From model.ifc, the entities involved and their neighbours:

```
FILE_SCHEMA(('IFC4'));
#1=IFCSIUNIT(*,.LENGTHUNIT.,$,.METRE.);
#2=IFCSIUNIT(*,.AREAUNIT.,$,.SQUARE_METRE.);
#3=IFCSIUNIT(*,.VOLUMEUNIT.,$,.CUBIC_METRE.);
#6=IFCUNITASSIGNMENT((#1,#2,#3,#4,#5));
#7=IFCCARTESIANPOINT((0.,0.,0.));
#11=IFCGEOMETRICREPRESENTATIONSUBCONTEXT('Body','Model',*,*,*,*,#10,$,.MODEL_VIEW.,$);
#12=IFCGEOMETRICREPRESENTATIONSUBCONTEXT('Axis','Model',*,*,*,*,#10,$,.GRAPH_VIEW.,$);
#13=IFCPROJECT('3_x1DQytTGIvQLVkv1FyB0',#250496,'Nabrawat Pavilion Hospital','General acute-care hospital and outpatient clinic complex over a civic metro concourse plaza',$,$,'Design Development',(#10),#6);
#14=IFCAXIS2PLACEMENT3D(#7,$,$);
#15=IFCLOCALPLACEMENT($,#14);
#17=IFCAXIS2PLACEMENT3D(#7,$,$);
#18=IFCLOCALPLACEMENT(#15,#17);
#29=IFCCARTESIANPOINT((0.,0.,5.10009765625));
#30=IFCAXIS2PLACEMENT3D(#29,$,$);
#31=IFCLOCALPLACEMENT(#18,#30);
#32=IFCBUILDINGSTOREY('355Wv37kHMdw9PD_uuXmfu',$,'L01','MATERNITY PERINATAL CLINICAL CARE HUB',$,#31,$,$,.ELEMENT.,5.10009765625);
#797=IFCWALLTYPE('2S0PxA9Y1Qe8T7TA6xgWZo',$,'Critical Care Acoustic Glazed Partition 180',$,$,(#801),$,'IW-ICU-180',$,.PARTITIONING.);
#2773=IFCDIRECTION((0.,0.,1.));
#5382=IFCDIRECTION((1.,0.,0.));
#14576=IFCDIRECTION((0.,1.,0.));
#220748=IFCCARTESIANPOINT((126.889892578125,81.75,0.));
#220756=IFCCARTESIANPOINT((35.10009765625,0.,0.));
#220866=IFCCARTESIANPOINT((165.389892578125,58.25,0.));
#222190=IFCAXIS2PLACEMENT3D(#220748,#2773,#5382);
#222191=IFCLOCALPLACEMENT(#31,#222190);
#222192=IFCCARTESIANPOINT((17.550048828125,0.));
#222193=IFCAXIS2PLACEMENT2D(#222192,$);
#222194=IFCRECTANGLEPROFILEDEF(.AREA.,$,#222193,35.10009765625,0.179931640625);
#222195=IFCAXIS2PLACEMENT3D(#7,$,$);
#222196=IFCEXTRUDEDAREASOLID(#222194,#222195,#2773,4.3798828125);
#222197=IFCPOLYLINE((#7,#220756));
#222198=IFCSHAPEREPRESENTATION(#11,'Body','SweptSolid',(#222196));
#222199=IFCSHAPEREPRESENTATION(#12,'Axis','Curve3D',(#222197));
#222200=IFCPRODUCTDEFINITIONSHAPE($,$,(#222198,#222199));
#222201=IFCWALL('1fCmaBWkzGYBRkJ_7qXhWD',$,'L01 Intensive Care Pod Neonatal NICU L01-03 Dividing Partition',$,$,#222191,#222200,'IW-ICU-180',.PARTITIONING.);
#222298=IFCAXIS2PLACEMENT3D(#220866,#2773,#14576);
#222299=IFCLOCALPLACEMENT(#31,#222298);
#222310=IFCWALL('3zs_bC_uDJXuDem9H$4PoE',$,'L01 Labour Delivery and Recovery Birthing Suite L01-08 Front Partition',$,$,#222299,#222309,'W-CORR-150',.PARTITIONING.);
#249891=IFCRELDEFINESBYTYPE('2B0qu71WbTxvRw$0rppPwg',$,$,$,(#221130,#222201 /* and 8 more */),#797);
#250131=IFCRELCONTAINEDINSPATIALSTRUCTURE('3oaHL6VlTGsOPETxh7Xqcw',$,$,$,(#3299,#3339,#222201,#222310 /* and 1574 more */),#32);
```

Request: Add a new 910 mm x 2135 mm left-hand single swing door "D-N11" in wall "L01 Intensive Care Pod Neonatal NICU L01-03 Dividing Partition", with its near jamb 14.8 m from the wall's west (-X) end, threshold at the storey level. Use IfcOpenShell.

```python
import numpy as np
import ifcopenshell
import ifcopenshell.api.feature
import ifcopenshell.api.geometry
import ifcopenshell.api.root
import ifcopenshell.api.spatial
import ifcopenshell.geom
import ifcopenshell.util.element
import ifcopenshell.util.placement
import ifcopenshell.util.representation
import ifcopenshell.util.shape
import ifcopenshell.util.unit

model = ifcopenshell.open("model.ifc")
unit_scale = ifcopenshell.util.unit.calculate_unit_scale(model)
settings = ifcopenshell.geom.settings()


def volume(element):
    """Net volume in cubic metres, openings subtracted."""
    shape = ifcopenshell.geom.create_shape(settings, element)
    return ifcopenshell.util.shape.get_volume(shape.geometry)


wall = model.by_guid("1fCmaBWkzGYBRkJ_7qXhWD")
storey = ifcopenshell.util.element.get_container(wall, ifc_class="IfcBuildingStorey")
context = ifcopenshell.util.representation.get_context(model, "Model", "Body", "MODEL_VIEW")
before = volume(wall)

width, height, from_end, sill = 0.91, 2.135, 14.8, 0.0  # metres

# The wall runs along its own X axis, and the end named is its -X end.
wall_shape = ifcopenshell.geom.create_shape(settings, wall)
x, y, z = ifcopenshell.util.shape.get_vertices(wall_shape.geometry).T
start = x.min() + from_end
face, thickness = float(y.min()), float(y.max() - y.min())
wall_matrix = ifcopenshell.util.placement.get_local_placement(wall.ObjectPlacement)
level = ifcopenshell.util.placement.get_local_placement(storey.ObjectPlacement)[2, 3]


def in_wall(x, y):
    """Placement at x, y metres in the wall's axes, at sill height."""
    matrix = wall_matrix.copy()
    matrix[:, 3] = wall_matrix @ np.array([x / unit_scale, y / unit_scale, 0.0, 1.0])
    matrix[2, 3] = level + sill / unit_scale
    return matrix


# Opening: a box that overshoots both wall faces by 50 mm.
opening = ifcopenshell.api.root.create_entity(model, ifc_class="IfcOpeningElement", predefined_type="OPENING")
box = ifcopenshell.api.geometry.add_wall_representation(
    model, context=context, length=width, height=height, thickness=thickness + 0.1
)
ifcopenshell.api.geometry.assign_representation(model, product=opening, representation=box)
ifcopenshell.api.geometry.edit_object_placement(model, product=opening, matrix=in_wall(start, face - 0.05), is_si=False)
ifcopenshell.api.feature.add_feature(model, feature=opening, element=wall)

door = ifcopenshell.api.root.create_entity(model, ifc_class="IfcDoor", name="D-N11", predefined_type="DOOR")
door.OverallWidth, door.OverallHeight = width / unit_scale, height / unit_scale
door.OperationType = "SINGLE_SWING_LEFT"
body = ifcopenshell.api.geometry.add_door_representation(
    model,
    context=context,
    overall_width=door.OverallWidth,
    overall_height=door.OverallHeight,
    operation_type="SINGLE_SWING_LEFT",
    lining_properties={"LiningDepth": thickness / unit_scale, "ThresholdDepth": thickness / unit_scale},
)
ifcopenshell.api.geometry.assign_representation(model, product=door, representation=body)
ifcopenshell.api.spatial.assign_container(model, products=[door], relating_structure=storey)
ifcopenshell.api.feature.add_filling(model, opening=opening, element=door)

# The lining spans the wall, so the door starts at the wall face.
ifcopenshell.api.geometry.edit_object_placement(model, product=door, matrix=in_wall(start, face), is_si=False)

after = volume(wall)

print(f"wall volume {before:.3f} -> {after:.3f} m3")

model.write("model_v2.ifc")
```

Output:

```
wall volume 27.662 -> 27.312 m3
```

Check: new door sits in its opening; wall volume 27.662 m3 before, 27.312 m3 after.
